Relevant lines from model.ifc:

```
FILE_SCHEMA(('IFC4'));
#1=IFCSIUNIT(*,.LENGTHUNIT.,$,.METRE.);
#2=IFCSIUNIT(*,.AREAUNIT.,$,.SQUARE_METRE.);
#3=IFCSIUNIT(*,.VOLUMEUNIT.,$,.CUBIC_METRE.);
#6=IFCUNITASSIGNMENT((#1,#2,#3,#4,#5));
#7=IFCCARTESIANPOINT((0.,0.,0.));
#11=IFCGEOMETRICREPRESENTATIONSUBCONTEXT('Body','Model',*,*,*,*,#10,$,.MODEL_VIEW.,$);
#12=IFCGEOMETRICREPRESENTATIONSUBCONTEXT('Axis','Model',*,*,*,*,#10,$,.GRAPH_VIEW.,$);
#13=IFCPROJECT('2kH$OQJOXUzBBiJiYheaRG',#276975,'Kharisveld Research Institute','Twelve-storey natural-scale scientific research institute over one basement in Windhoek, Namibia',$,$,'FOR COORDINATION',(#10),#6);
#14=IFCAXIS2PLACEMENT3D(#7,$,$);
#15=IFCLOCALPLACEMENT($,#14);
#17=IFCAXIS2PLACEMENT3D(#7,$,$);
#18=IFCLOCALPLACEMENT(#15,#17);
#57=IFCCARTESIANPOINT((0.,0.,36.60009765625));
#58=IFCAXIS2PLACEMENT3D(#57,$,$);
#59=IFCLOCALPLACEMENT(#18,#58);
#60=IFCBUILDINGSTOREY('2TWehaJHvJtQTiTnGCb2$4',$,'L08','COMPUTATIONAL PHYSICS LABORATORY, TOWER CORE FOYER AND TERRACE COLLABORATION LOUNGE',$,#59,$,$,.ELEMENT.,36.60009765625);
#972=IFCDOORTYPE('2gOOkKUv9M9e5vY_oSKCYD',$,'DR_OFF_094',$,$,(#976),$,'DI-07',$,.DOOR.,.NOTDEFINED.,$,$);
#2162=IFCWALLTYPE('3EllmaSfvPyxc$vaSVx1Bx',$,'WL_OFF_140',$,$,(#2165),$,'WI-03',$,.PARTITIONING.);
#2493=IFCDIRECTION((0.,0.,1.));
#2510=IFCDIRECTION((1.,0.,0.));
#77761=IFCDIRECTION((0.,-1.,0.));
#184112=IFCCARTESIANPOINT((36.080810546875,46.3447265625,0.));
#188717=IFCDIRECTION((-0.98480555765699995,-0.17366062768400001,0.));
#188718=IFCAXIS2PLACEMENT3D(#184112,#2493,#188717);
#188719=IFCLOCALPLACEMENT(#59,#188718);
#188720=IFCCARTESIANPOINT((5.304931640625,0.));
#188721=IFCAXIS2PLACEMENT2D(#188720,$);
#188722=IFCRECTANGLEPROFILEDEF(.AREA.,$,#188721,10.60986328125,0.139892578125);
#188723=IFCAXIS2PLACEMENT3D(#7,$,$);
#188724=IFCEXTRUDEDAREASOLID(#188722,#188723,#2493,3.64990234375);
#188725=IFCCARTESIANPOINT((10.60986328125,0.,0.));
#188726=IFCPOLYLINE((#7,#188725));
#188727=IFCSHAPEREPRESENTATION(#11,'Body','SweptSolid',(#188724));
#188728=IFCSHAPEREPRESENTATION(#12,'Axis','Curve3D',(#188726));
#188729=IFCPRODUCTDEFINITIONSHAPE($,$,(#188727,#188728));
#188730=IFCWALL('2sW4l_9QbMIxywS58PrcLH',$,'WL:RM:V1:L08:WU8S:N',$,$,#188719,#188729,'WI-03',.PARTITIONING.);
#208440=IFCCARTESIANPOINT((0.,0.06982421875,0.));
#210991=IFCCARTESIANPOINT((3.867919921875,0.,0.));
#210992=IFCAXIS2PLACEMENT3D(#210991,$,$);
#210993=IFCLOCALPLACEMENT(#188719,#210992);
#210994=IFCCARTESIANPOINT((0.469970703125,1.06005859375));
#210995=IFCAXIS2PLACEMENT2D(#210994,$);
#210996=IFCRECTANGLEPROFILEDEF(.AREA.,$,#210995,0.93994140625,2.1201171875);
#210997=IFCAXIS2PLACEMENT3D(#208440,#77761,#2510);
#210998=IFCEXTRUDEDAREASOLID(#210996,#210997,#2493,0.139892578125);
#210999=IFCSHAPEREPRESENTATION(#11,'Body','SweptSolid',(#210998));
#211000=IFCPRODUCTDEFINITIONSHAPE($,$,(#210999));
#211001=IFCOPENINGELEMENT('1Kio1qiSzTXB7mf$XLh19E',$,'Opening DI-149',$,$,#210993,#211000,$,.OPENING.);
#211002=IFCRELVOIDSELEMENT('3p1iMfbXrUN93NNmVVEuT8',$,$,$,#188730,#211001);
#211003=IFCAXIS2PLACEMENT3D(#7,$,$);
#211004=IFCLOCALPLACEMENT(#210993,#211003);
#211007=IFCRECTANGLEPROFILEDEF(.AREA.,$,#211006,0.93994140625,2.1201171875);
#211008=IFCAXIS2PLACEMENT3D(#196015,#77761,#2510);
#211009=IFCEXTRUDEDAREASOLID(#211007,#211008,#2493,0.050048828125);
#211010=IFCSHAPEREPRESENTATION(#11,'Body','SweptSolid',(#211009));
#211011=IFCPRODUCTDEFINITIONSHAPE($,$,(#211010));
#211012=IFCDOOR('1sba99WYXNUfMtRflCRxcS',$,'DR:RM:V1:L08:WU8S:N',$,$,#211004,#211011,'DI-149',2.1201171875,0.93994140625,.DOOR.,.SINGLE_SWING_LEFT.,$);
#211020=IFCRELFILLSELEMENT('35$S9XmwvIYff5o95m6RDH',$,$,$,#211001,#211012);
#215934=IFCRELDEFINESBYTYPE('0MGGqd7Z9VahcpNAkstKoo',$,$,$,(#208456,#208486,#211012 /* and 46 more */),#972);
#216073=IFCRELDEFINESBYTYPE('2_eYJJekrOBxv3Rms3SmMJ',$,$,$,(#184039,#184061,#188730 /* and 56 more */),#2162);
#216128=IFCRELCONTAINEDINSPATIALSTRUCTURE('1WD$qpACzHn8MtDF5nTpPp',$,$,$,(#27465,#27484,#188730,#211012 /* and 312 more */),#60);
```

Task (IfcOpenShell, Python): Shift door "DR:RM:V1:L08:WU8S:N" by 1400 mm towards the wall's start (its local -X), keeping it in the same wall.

```python
import ifcopenshell
import ifcopenshell.api.geometry
import ifcopenshell.util.placement
import ifcopenshell.util.unit

model = ifcopenshell.open("model.ifc")
unit_scale = ifcopenshell.util.unit.calculate_unit_scale(model)

door = model.by_guid("1sba99WYXNUfMtRflCRxcS")
opening = door.FillsVoids[0].RelatingOpeningElement
wall = opening.VoidsElements[0].RelatingBuildingElement

wall_matrix = ifcopenshell.util.placement.get_local_placement(wall.ObjectPlacement)
shift = wall_matrix[:3, 0] * -1.4 / unit_scale
before = ifcopenshell.util.placement.get_local_placement(door.ObjectPlacement)[:3, 3].copy()

# The door is placed relative to its opening, so it follows when the opening moves.
matrix = ifcopenshell.util.placement.get_local_placement(opening.ObjectPlacement)
matrix[:3, 3] += shift
ifcopenshell.api.geometry.edit_object_placement(
    model, product=opening, matrix=matrix, is_si=False, should_transform_children=True
)

after = ifcopenshell.util.placement.get_local_placement(door.ObjectPlacement)[:3, 3]
print("door moved by", (after - before).round(3) + 0.0)

model.write("model_updated.ifc")
```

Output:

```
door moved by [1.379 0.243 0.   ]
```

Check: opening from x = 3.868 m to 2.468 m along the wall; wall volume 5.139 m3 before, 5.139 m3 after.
